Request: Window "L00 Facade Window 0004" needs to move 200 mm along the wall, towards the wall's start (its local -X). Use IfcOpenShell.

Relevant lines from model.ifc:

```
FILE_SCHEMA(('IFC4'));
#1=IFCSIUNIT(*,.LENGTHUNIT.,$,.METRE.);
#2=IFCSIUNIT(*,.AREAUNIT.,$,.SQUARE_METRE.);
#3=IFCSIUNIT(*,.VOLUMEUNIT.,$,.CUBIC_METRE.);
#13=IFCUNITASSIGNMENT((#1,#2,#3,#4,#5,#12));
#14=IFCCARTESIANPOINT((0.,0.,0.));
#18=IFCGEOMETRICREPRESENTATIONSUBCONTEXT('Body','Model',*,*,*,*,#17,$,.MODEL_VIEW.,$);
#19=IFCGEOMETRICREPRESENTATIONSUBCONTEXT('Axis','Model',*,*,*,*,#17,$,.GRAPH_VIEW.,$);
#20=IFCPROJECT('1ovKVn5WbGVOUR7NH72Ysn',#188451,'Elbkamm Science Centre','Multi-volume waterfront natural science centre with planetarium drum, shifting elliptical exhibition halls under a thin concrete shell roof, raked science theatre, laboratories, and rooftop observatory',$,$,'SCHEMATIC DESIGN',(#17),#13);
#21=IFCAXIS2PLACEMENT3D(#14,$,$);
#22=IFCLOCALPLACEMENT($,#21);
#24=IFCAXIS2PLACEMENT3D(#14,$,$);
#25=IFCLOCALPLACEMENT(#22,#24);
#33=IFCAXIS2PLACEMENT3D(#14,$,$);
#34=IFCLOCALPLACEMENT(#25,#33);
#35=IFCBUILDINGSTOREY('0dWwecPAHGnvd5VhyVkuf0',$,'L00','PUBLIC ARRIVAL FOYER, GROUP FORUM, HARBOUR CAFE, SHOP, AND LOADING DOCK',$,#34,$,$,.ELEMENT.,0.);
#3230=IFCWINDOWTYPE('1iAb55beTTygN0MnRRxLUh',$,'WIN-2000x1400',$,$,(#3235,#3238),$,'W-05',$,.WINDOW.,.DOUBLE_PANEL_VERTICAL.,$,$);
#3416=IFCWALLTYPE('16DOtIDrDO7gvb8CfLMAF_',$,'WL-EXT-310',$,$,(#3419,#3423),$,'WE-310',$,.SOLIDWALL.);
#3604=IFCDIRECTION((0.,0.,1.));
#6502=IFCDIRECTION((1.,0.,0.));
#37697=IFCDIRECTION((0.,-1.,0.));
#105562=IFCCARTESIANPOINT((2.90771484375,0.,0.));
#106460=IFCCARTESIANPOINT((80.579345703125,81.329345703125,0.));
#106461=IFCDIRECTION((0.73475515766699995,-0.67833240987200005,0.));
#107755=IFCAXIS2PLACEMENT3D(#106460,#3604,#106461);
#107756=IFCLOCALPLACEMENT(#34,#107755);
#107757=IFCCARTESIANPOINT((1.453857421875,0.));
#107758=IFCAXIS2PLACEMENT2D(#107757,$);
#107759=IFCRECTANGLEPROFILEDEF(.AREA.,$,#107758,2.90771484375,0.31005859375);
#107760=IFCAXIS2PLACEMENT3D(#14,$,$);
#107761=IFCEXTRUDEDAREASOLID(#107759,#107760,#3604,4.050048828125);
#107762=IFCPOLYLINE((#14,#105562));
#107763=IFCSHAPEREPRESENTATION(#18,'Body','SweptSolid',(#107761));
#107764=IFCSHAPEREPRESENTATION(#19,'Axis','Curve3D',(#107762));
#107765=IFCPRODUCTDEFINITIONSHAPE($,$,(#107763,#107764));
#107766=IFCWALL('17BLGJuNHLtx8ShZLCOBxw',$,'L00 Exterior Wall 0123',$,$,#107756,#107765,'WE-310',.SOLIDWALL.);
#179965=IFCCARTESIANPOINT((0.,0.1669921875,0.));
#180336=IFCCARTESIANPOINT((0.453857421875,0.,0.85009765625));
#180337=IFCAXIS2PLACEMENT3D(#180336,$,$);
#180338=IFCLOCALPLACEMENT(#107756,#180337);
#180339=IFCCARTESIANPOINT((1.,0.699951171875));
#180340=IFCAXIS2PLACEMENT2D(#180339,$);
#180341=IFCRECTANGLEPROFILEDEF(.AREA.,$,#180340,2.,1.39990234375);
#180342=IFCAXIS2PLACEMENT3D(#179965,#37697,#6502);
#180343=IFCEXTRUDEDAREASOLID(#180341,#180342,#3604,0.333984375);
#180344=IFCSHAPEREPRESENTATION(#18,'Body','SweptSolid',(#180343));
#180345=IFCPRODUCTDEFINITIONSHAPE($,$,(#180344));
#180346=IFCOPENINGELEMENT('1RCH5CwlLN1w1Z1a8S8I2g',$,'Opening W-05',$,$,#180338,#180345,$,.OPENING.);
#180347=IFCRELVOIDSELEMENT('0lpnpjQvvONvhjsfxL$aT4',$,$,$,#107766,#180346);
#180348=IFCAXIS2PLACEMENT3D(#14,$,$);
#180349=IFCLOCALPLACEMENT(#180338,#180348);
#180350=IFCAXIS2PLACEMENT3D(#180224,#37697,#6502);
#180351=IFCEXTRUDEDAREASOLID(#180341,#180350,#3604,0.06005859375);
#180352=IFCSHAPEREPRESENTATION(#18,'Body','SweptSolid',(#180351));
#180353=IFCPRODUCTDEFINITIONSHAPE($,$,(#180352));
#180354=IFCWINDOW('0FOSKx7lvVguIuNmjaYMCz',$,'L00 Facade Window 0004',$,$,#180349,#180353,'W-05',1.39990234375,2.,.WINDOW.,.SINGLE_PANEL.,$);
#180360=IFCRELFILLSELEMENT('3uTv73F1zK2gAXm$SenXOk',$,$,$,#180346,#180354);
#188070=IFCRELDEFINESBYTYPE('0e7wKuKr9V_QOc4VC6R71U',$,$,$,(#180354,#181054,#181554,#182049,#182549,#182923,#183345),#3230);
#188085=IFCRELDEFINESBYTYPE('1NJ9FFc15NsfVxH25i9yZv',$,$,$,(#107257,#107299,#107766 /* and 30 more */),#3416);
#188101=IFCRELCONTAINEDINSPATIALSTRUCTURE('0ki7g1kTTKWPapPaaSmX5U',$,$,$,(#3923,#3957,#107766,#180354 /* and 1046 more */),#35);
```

```python
import ifcopenshell
import ifcopenshell.api.geometry
import ifcopenshell.util.placement
import ifcopenshell.util.unit

model = ifcopenshell.open("model.ifc")
unit_scale = ifcopenshell.util.unit.calculate_unit_scale(model)

window = model.by_guid("0FOSKx7lvVguIuNmjaYMCz")
opening = window.FillsVoids[0].RelatingOpeningElement
wall = opening.VoidsElements[0].RelatingBuildingElement

wall_matrix = ifcopenshell.util.placement.get_local_placement(wall.ObjectPlacement)
shift = wall_matrix[:3, 0] * -0.2 / unit_scale
before = ifcopenshell.util.placement.get_local_placement(window.ObjectPlacement)[:3, 3].copy()

# The window is placed relative to its opening, so it follows when the opening moves.
matrix = ifcopenshell.util.placement.get_local_placement(opening.ObjectPlacement)
matrix[:3, 3] += shift
ifcopenshell.api.geometry.edit_object_placement(
    model, product=opening, matrix=matrix, is_si=False, should_transform_children=True
)

after = ifcopenshell.util.placement.get_local_placement(window.ObjectPlacement)[:3, 3]
print("window moved by", (after - before).round(3) + 0.0)

model.write("model-out.ifc")
```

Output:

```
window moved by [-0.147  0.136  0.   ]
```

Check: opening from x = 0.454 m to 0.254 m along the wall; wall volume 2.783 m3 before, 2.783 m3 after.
